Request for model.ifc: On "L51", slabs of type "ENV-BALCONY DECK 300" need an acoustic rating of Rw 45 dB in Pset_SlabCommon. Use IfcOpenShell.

First a look at what the model holds.

```python
import ifcopenshell
import ifcopenshell.util.element

model = ifcopenshell.open("model.ifc")
print(model.schema)
storey = next(s for s in model.by_type("IfcBuildingStorey") if s.Name == "L51")
slabs = [e for e in ifcopenshell.util.element.get_decomposition(storey) if e.is_a("IfcSlab")]
seen = {}
for e in slabs:
    element_type = ifcopenshell.util.element.get_type(e)
    key = (element_type.Name if element_type != e and element_type else None, ifcopenshell.util.element.get_pset(e, "Pset_SlabCommon", "AcousticRating"))
    seen[key] = seen.get(key, 0) + 1
for (name, value), count in sorted(seen.items(), key=str):
    print(count, "x", name, "|", value)
```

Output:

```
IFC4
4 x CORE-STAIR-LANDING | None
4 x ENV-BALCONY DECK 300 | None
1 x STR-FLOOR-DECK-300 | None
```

```python
import ifcopenshell
import ifcopenshell.api.pset
import ifcopenshell.util.element

model = ifcopenshell.open("model.ifc")

storey = next(s for s in model.by_type("IfcBuildingStorey") if s.Name == "L51")
slabs = [e for e in ifcopenshell.util.element.get_decomposition(storey) if e.is_a("IfcSlab")]

count = 0
for e in slabs:
    element_type = ifcopenshell.util.element.get_type(e)
    if element_type in (None, e) or element_type.Name != "ENV-BALCONY DECK 300":
        continue
    found = ifcopenshell.util.element.get_pset(e, "Pset_SlabCommon", should_inherit=False)
    if found:
        pset = model.by_id(found["id"])
        if len(ifcopenshell.util.element.get_elements_by_pset(pset)) > 1:
            pset = ifcopenshell.api.pset.unshare_pset(model, products=[e], pset=pset)[0]
    else:
        pset = ifcopenshell.api.pset.add_pset(model, product=e, name="Pset_SlabCommon")
    ifcopenshell.api.pset.edit_pset(model, pset=pset, properties={"AcousticRating": "Rw 45 dB"})
    count += 1

print(count, "slabs updated")

model.write("model_edited.ifc")
```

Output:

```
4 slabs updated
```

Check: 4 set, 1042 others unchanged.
